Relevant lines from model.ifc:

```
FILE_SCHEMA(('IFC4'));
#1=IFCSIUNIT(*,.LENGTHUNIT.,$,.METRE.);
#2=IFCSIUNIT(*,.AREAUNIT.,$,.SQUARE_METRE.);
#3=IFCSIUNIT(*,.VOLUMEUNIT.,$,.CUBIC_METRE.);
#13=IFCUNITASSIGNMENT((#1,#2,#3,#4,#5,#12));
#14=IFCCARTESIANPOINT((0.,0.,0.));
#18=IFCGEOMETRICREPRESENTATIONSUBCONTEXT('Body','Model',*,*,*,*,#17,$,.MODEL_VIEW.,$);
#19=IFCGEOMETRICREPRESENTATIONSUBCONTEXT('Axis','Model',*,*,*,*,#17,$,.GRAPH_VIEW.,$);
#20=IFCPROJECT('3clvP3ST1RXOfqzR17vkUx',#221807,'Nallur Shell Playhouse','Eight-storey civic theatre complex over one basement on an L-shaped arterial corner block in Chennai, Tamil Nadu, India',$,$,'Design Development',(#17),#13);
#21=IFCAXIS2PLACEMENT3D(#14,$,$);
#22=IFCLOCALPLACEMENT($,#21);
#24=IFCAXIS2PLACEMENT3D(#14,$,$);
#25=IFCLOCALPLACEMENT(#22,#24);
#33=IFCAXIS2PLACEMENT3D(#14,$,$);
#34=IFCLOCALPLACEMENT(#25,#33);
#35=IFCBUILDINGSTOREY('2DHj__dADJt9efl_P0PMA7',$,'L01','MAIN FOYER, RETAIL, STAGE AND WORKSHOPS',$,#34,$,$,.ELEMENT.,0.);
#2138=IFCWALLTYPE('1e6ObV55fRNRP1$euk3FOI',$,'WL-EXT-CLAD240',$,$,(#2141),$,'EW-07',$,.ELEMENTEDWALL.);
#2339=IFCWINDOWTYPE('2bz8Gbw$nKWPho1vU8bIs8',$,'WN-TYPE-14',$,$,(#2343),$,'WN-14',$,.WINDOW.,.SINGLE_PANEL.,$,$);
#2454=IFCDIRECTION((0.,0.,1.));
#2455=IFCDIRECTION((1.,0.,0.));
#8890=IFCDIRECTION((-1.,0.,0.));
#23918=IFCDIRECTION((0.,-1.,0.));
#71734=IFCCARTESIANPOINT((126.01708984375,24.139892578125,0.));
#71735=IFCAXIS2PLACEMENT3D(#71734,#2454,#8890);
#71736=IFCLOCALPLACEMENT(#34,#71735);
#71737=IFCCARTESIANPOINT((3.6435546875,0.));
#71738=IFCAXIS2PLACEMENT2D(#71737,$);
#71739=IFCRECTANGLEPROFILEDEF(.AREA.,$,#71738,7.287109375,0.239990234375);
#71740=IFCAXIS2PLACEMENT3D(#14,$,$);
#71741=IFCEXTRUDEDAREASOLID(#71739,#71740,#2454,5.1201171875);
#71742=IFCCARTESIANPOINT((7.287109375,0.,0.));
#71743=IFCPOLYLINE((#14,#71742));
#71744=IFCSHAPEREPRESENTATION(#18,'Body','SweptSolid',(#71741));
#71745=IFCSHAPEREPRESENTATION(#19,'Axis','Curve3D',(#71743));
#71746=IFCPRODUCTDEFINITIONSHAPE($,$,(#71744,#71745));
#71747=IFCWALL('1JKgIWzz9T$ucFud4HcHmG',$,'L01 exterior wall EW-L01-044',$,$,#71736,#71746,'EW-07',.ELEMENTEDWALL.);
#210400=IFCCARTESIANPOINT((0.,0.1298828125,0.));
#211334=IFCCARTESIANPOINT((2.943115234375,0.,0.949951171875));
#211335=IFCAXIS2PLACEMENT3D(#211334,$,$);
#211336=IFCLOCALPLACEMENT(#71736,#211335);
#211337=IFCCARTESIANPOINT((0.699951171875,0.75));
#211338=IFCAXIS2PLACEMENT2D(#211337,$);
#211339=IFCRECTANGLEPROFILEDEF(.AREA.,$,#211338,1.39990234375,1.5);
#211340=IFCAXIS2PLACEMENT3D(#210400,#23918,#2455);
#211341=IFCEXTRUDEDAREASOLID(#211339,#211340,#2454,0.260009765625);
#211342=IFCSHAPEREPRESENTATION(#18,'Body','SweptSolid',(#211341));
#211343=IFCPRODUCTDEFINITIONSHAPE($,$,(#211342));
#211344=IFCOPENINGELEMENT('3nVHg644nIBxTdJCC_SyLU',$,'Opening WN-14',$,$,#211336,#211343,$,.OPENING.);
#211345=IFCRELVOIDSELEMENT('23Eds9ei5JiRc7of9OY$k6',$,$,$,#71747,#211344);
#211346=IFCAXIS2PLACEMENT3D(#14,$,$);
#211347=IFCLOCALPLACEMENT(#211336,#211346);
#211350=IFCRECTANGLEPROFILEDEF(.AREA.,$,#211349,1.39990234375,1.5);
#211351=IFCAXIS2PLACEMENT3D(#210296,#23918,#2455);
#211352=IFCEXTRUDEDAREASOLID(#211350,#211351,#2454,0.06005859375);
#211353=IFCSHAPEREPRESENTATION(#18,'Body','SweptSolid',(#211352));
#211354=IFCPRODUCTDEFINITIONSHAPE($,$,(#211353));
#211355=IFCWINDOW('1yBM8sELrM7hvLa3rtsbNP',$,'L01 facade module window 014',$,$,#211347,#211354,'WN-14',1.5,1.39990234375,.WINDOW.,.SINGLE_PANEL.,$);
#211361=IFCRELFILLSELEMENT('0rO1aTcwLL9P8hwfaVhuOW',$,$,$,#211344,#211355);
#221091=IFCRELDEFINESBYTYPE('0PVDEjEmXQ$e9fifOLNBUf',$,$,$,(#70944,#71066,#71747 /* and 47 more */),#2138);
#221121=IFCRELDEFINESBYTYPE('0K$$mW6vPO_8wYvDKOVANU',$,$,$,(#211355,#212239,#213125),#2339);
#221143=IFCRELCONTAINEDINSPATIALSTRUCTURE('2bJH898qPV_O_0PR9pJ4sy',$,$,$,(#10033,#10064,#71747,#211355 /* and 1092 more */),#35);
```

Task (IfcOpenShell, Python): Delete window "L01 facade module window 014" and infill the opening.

```python
import ifcopenshell
import ifcopenshell.api.feature
import ifcopenshell.api.root
import ifcopenshell.geom
import ifcopenshell.util.shape

model = ifcopenshell.open("model.ifc")
settings = ifcopenshell.geom.settings()


def volume(element):
    """Net volume in cubic metres, openings subtracted."""
    shape = ifcopenshell.geom.create_shape(settings, element)
    return ifcopenshell.util.shape.get_volume(shape.geometry)


window = model.by_guid("1yBM8sELrM7hvLa3rtsbNP")
opening = window.FillsVoids[0].RelatingOpeningElement
wall = opening.VoidsElements[0].RelatingBuildingElement
before = volume(wall)

ifcopenshell.api.root.remove_product(model, product=window)
ifcopenshell.api.feature.remove_feature(model, feature=opening)

after = volume(wall)

print(f"wall volume {before:.3f} -> {after:.3f} m3")

model.write("model_v2.ifc")
```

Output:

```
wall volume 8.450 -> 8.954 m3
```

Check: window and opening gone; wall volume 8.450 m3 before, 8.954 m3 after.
